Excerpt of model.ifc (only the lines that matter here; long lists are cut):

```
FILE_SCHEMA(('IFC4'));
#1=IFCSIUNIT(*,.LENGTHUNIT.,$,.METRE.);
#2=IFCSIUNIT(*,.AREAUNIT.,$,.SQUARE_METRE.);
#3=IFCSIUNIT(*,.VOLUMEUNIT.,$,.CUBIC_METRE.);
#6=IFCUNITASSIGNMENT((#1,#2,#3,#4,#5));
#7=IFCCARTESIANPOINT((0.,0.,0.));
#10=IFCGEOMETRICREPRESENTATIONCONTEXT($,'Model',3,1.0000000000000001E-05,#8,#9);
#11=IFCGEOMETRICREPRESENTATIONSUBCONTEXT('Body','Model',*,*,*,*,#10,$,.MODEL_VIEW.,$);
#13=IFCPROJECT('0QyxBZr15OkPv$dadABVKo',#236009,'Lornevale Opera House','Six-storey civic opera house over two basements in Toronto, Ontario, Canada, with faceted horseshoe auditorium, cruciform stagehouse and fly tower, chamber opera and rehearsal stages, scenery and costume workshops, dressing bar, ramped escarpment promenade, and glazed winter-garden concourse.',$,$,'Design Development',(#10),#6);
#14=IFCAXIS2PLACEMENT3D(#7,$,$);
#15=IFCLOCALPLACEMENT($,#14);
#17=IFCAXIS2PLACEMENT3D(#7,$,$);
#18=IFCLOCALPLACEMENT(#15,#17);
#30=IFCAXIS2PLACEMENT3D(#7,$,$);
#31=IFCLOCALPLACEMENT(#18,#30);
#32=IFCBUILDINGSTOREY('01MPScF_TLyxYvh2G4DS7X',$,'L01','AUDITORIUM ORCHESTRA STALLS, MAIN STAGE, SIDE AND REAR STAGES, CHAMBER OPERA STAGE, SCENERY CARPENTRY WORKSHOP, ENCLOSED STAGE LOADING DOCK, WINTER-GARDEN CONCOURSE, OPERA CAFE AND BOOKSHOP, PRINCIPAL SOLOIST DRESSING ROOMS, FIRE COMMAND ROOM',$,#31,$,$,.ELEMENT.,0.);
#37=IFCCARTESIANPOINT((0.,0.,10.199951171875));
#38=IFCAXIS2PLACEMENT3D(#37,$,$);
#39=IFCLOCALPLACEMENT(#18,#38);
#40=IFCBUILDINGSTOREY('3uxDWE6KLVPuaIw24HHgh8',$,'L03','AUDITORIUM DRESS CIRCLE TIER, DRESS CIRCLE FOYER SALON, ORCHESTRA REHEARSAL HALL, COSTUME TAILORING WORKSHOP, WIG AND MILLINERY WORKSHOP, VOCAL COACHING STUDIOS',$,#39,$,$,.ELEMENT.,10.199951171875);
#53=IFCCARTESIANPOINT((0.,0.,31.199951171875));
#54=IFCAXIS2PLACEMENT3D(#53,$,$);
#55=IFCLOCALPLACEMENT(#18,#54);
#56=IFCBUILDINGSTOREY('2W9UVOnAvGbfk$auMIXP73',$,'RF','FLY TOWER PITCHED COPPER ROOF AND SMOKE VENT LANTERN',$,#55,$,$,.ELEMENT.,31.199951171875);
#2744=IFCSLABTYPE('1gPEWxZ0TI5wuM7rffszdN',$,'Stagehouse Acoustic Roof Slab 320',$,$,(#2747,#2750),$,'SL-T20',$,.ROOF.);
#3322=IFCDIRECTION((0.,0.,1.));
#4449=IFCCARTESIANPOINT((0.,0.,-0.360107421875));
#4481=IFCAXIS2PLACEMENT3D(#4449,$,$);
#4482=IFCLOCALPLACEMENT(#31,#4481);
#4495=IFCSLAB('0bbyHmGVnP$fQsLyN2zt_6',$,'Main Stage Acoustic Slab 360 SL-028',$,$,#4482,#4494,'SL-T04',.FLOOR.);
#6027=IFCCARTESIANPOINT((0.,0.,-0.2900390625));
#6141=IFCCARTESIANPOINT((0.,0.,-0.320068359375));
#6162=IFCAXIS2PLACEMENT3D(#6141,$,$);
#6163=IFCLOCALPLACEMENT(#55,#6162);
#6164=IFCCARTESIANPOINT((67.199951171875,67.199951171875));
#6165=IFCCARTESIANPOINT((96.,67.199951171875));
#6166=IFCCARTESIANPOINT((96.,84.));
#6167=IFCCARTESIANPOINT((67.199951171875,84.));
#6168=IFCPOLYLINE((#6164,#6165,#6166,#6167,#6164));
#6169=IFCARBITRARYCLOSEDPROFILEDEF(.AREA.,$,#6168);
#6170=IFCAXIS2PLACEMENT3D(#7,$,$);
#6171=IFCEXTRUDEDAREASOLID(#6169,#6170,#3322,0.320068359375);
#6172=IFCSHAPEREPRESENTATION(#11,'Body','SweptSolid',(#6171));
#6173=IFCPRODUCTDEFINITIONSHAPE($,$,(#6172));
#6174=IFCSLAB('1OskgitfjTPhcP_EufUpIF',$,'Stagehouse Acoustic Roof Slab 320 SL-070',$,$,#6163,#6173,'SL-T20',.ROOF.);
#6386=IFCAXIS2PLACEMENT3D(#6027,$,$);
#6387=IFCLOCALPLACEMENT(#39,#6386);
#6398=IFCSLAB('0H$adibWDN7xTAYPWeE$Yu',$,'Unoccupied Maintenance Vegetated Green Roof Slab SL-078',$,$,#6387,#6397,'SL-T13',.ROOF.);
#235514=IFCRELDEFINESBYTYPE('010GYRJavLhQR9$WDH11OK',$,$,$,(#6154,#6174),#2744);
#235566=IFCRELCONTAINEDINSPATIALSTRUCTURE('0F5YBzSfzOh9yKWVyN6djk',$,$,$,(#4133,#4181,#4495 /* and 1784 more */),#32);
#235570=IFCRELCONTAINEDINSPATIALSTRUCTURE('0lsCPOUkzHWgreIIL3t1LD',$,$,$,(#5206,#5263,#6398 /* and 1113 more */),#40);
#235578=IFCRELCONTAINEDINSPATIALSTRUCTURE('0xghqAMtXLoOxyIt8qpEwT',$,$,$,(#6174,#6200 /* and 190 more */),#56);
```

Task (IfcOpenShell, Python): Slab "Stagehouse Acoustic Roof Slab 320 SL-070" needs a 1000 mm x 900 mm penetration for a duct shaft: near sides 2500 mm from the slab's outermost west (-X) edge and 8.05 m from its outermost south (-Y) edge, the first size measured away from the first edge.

```python
import numpy as np
import ifcopenshell
import ifcopenshell.api.feature
import ifcopenshell.api.geometry
import ifcopenshell.api.root
import ifcopenshell.geom
import ifcopenshell.util.placement
import ifcopenshell.util.representation
import ifcopenshell.util.shape
import ifcopenshell.util.unit

model = ifcopenshell.open("model.ifc")
unit_scale = ifcopenshell.util.unit.calculate_unit_scale(model)
settings = ifcopenshell.geom.settings()


def volume(element):
    """Net volume in cubic metres, openings subtracted."""
    shape = ifcopenshell.geom.create_shape(settings, element)
    return ifcopenshell.util.shape.get_volume(shape.geometry)


slab = model.by_guid("1OskgitfjTPhcP_EufUpIF")
before = volume(slab)

# Extent in the slab's own axes, in metres. The edges named are its -X and -Y sides.
slab_shape = ifcopenshell.geom.create_shape(settings, slab)
vertices = ifcopenshell.util.shape.get_vertices(slab_shape.geometry)
x_min, y_min, bottom = vertices.min(axis=0)
top = vertices[:, 2].max()

opening = ifcopenshell.api.root.create_entity(model, ifc_class="IfcOpeningElement", name="Duct shaft opening", predefined_type="OPENING")
context = ifcopenshell.util.representation.get_context(model, "Model", "Body", "MODEL_VIEW")
width, depth = 1, 0.9
outline = [(0.0, 0.0), (width, 0.0), (width, depth), (0.0, depth), (0.0, 0.0)]
# Overshoot both faces by 50 mm so the cut is clean.
shape = ifcopenshell.api.geometry.add_slab_representation(
    model, context=context, depth=top - bottom + 0.1, polyline=outline
)
ifcopenshell.api.geometry.assign_representation(model, product=opening, representation=shape)

matrix = ifcopenshell.util.placement.get_local_placement(slab.ObjectPlacement)
matrix[:, 3] = matrix @ np.append(np.array([x_min + 2.5, y_min + 8.05, bottom - 0.05]) / unit_scale, 1.0)
ifcopenshell.api.geometry.edit_object_placement(model, product=opening, matrix=matrix, is_si=False)
ifcopenshell.api.feature.add_feature(model, feature=opening, element=slab)

after = volume(slab)

print(f"slab volume {before:.3f} -> {after:.3f} m3")

model.write("model_v2.ifc")
```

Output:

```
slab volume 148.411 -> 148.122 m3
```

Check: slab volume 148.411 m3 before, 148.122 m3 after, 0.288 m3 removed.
